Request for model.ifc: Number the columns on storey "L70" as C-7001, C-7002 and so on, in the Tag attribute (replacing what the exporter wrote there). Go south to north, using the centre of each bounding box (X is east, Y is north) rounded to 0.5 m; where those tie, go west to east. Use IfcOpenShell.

First a look at what the model holds.

```python
import ifcopenshell
import ifcopenshell.util.element
import ifcopenshell.util.placement

model = ifcopenshell.open("model.ifc")
print(model.schema)
storey = next(s for s in model.by_type("IfcBuildingStorey") if s.Name == "L70")
columns = [e for e in ifcopenshell.util.element.get_decomposition(storey) if e.is_a("IfcColumn")]
for e in sorted(columns, key=lambda e: e.id()):
    origin = ifcopenshell.util.placement.get_local_placement(e.ObjectPlacement)[:3, 3]
    print(e.id(), e.Tag, e.Name, origin.round(2) + 0.0, sep=" | ")
```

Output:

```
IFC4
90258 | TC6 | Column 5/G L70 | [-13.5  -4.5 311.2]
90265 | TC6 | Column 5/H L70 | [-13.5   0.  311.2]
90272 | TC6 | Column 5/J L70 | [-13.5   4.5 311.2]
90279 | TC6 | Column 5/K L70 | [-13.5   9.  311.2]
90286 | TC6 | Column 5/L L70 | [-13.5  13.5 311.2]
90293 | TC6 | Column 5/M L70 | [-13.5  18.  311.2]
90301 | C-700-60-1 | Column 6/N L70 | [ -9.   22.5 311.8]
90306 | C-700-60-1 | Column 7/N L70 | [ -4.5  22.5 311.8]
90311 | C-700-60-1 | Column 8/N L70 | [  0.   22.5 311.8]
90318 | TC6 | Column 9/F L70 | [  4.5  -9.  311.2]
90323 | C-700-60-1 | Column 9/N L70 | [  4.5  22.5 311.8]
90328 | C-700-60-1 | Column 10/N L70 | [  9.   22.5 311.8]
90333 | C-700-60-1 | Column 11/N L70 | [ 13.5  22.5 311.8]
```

```python
import ifcopenshell
import ifcopenshell.geom
import ifcopenshell.util.element
import ifcopenshell.util.shape

model = ifcopenshell.open("model.ifc")
settings = ifcopenshell.geom.settings()
settings.set("use-world-coords", True)


def centre(element):
    shape = ifcopenshell.geom.create_shape(settings, element)
    return ifcopenshell.util.shape.get_bbox_centroid(shape.geometry)


storey = next(s for s in model.by_type("IfcBuildingStorey") if s.Name == "L70")
columns = [e for e in ifcopenshell.util.element.get_decomposition(storey) if e.is_a("IfcColumn")]

# Insertion points can sit at a corner or the storey origin, so sort by the geometry (in metres).
centres = {e: centre(e) for e in columns}
columns.sort(key=lambda e: (round(centres[e][1] / 0.5), centres[e][0]))

for i, e in enumerate(columns, start=1):
    number = f"C-70{i:02d}"
    e.Tag = number
    print(e.id(), number)

model.write("model_v2.ifc")
```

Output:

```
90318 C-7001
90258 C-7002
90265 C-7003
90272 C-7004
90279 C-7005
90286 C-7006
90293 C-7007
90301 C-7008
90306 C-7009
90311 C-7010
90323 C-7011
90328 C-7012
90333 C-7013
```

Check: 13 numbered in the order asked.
